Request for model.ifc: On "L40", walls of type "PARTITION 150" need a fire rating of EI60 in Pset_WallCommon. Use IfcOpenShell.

First a look at what the model holds.

```python
import ifcopenshell
import ifcopenshell.util.element

model = ifcopenshell.open("model.ifc")
print(model.schema)
storey = next(s for s in model.by_type("IfcBuildingStorey") if s.Name == "L40")
walls = [e for e in ifcopenshell.util.element.get_decomposition(storey) if e.is_a("IfcWall")]
seen = {}
for e in walls:
    element_type = ifcopenshell.util.element.get_type(e)
    key = (element_type.Name if element_type != e and element_type else None, ifcopenshell.util.element.get_pset(e, "Pset_WallCommon", "FireRating"))
    seen[key] = seen.get(key, 0) + 1
for (name, value), count in sorted(seen.items(), key=str):
    print(count, "x", name, "|", value)
```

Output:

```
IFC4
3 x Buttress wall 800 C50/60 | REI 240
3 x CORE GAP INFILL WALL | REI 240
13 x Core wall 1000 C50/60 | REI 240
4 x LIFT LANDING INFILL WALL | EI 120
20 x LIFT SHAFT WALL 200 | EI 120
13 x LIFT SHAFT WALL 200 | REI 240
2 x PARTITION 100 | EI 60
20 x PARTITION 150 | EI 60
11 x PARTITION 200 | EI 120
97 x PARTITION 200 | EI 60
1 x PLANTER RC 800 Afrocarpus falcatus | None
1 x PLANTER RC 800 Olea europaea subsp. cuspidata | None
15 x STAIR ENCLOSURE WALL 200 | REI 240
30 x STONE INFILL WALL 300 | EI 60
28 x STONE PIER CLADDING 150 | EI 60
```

```python
import ifcopenshell
import ifcopenshell.api.pset
import ifcopenshell.util.element

model = ifcopenshell.open("model.ifc")

storey = next(s for s in model.by_type("IfcBuildingStorey") if s.Name == "L40")
walls = [e for e in ifcopenshell.util.element.get_decomposition(storey) if e.is_a("IfcWall")]

count = 0
for e in walls:
    element_type = ifcopenshell.util.element.get_type(e)
    if element_type in (None, e) or element_type.Name != "PARTITION 150":
        continue
    found = ifcopenshell.util.element.get_pset(e, "Pset_WallCommon", should_inherit=False)
    if found:
        pset = model.by_id(found["id"])
        if len(ifcopenshell.util.element.get_elements_by_pset(pset)) > 1:
            pset = ifcopenshell.api.pset.unshare_pset(model, products=[e], pset=pset)[0]
    else:
        pset = ifcopenshell.api.pset.add_pset(model, product=e, name="Pset_WallCommon")
    ifcopenshell.api.pset.edit_pset(model, pset=pset, properties={"FireRating": "EI60"})
    count += 1

print(count, "walls updated")

model.write("model-out.ifc")
```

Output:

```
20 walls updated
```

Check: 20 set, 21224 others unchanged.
